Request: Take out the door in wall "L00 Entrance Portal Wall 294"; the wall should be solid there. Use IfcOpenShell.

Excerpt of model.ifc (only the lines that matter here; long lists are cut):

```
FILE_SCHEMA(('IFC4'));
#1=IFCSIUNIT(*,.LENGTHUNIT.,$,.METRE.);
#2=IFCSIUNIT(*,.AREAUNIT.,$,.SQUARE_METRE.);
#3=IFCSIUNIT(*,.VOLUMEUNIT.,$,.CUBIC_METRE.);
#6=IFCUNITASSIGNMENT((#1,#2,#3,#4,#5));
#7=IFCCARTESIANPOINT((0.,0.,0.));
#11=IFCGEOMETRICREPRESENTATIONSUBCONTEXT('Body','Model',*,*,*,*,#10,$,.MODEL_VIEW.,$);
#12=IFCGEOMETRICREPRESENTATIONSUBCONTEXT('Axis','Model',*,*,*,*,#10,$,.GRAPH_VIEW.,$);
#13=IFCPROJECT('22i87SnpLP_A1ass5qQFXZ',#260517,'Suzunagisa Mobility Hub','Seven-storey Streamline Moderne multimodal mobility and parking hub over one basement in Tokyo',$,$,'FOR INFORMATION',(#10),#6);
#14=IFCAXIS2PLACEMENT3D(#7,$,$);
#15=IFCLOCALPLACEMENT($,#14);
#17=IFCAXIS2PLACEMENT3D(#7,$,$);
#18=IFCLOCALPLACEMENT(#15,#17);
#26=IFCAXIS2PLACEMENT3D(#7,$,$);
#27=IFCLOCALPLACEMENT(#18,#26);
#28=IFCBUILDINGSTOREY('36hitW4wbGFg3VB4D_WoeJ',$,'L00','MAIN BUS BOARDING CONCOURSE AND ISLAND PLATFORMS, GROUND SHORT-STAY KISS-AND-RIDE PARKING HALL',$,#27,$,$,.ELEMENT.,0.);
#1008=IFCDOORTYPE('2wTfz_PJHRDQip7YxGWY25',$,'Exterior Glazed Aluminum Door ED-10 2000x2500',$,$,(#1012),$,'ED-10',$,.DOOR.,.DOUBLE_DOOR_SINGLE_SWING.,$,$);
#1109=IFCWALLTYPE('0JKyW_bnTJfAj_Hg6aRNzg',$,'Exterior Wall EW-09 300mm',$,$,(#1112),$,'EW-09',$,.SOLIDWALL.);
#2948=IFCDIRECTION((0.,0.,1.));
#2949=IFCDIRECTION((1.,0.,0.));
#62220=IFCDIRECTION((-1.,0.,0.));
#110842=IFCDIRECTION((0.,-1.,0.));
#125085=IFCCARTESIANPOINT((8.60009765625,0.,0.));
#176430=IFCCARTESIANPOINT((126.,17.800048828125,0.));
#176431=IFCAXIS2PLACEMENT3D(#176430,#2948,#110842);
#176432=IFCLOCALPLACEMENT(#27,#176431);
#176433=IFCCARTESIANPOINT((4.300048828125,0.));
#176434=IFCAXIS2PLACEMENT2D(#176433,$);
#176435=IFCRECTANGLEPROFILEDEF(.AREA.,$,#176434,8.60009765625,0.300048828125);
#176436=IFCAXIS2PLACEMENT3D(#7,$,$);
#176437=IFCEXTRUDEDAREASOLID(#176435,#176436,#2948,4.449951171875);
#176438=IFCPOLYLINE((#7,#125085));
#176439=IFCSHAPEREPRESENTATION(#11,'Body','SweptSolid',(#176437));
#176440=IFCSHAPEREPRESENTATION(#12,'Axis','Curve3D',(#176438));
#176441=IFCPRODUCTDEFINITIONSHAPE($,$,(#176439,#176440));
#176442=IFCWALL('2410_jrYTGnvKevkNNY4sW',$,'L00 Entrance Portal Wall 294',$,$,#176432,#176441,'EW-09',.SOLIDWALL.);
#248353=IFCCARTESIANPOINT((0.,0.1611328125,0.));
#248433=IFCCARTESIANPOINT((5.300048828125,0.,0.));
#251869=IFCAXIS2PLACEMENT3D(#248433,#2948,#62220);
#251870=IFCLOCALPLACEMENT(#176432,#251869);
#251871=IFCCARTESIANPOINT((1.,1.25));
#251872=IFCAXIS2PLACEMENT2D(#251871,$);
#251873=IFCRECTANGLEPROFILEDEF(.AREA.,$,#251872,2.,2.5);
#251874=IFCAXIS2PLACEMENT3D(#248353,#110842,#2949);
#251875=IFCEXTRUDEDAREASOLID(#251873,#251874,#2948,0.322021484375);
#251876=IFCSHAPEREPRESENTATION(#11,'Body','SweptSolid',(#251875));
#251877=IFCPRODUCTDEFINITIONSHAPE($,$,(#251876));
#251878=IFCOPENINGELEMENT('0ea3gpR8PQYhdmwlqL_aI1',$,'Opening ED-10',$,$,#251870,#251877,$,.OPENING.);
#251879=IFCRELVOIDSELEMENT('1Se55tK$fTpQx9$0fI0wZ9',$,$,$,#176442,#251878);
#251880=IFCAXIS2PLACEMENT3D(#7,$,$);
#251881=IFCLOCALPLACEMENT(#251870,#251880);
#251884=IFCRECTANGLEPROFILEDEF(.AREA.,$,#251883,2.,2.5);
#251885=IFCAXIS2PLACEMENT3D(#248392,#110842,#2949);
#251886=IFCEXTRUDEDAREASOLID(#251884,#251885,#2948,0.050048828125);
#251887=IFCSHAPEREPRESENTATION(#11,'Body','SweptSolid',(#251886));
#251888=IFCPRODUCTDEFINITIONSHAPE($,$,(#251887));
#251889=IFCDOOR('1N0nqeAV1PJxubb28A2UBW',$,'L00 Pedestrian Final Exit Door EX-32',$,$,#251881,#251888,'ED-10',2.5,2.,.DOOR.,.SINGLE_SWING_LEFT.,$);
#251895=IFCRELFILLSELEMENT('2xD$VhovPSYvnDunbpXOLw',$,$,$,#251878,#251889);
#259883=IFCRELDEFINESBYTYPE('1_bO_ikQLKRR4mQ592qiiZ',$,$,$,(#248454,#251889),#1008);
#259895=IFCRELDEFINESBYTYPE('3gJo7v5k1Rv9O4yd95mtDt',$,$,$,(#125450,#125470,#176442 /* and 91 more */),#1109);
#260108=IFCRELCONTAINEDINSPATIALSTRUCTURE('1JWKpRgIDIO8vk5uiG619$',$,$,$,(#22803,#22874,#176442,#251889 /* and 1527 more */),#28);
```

```python
import ifcopenshell
import ifcopenshell.api.feature
import ifcopenshell.api.root
import ifcopenshell.geom
import ifcopenshell.util.shape

model = ifcopenshell.open("model.ifc")
settings = ifcopenshell.geom.settings()


def volume(element):
    """Net volume in cubic metres, openings subtracted."""
    shape = ifcopenshell.geom.create_shape(settings, element)
    return ifcopenshell.util.shape.get_volume(shape.geometry)


door = model.by_guid("1N0nqeAV1PJxubb28A2UBW")
opening = door.FillsVoids[0].RelatingOpeningElement
wall = opening.VoidsElements[0].RelatingBuildingElement
before = volume(wall)

ifcopenshell.api.root.remove_product(model, product=door)
ifcopenshell.api.feature.remove_feature(model, feature=opening)

after = volume(wall)

print(f"wall volume {before:.3f} -> {after:.3f} m3")

model.write("model_v2.ifc")
```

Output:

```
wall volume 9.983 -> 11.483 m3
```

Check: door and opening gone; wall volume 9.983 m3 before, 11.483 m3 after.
